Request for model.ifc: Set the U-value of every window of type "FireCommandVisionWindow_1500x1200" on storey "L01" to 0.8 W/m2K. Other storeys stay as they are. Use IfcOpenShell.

First a look at what the model holds.

```python
import ifcopenshell
import ifcopenshell.util.element

model = ifcopenshell.open("model.ifc")
print(model.schema)
storey = next(s for s in model.by_type("IfcBuildingStorey") if s.Name == "L01")
windows = [e for e in ifcopenshell.util.element.get_decomposition(storey) if e.is_a("IfcWindow")]
seen = {}
for e in windows:
    element_type = ifcopenshell.util.element.get_type(e)
    key = (element_type.Name if element_type != e and element_type else None, ifcopenshell.util.element.get_pset(e, "Pset_WindowCommon", "ThermalTransmittance"))
    seen[key] = seen.get(key, 0) + 1
for (name, value), count in sorted(seen.items(), key=str):
    print(count, "x", name, "|", value)
```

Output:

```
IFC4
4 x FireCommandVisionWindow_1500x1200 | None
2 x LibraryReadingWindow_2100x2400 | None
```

```python
import ifcopenshell
import ifcopenshell.api.pset
import ifcopenshell.util.element

model = ifcopenshell.open("model.ifc")

storey = next(s for s in model.by_type("IfcBuildingStorey") if s.Name == "L01")
windows = [e for e in ifcopenshell.util.element.get_decomposition(storey) if e.is_a("IfcWindow")]

count = 0
for e in windows:
    element_type = ifcopenshell.util.element.get_type(e)
    if element_type in (None, e) or element_type.Name != "FireCommandVisionWindow_1500x1200":
        continue
    # add_pset returns the element's existing set when there is one.
    pset = ifcopenshell.api.pset.add_pset(model, product=e, name="Pset_WindowCommon")
    ifcopenshell.api.pset.edit_pset(model, pset=pset, properties={"ThermalTransmittance": 0.8})
    count += 1

print(count, "windows updated")

model.write("model-out.ifc")
```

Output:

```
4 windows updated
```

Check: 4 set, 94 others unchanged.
